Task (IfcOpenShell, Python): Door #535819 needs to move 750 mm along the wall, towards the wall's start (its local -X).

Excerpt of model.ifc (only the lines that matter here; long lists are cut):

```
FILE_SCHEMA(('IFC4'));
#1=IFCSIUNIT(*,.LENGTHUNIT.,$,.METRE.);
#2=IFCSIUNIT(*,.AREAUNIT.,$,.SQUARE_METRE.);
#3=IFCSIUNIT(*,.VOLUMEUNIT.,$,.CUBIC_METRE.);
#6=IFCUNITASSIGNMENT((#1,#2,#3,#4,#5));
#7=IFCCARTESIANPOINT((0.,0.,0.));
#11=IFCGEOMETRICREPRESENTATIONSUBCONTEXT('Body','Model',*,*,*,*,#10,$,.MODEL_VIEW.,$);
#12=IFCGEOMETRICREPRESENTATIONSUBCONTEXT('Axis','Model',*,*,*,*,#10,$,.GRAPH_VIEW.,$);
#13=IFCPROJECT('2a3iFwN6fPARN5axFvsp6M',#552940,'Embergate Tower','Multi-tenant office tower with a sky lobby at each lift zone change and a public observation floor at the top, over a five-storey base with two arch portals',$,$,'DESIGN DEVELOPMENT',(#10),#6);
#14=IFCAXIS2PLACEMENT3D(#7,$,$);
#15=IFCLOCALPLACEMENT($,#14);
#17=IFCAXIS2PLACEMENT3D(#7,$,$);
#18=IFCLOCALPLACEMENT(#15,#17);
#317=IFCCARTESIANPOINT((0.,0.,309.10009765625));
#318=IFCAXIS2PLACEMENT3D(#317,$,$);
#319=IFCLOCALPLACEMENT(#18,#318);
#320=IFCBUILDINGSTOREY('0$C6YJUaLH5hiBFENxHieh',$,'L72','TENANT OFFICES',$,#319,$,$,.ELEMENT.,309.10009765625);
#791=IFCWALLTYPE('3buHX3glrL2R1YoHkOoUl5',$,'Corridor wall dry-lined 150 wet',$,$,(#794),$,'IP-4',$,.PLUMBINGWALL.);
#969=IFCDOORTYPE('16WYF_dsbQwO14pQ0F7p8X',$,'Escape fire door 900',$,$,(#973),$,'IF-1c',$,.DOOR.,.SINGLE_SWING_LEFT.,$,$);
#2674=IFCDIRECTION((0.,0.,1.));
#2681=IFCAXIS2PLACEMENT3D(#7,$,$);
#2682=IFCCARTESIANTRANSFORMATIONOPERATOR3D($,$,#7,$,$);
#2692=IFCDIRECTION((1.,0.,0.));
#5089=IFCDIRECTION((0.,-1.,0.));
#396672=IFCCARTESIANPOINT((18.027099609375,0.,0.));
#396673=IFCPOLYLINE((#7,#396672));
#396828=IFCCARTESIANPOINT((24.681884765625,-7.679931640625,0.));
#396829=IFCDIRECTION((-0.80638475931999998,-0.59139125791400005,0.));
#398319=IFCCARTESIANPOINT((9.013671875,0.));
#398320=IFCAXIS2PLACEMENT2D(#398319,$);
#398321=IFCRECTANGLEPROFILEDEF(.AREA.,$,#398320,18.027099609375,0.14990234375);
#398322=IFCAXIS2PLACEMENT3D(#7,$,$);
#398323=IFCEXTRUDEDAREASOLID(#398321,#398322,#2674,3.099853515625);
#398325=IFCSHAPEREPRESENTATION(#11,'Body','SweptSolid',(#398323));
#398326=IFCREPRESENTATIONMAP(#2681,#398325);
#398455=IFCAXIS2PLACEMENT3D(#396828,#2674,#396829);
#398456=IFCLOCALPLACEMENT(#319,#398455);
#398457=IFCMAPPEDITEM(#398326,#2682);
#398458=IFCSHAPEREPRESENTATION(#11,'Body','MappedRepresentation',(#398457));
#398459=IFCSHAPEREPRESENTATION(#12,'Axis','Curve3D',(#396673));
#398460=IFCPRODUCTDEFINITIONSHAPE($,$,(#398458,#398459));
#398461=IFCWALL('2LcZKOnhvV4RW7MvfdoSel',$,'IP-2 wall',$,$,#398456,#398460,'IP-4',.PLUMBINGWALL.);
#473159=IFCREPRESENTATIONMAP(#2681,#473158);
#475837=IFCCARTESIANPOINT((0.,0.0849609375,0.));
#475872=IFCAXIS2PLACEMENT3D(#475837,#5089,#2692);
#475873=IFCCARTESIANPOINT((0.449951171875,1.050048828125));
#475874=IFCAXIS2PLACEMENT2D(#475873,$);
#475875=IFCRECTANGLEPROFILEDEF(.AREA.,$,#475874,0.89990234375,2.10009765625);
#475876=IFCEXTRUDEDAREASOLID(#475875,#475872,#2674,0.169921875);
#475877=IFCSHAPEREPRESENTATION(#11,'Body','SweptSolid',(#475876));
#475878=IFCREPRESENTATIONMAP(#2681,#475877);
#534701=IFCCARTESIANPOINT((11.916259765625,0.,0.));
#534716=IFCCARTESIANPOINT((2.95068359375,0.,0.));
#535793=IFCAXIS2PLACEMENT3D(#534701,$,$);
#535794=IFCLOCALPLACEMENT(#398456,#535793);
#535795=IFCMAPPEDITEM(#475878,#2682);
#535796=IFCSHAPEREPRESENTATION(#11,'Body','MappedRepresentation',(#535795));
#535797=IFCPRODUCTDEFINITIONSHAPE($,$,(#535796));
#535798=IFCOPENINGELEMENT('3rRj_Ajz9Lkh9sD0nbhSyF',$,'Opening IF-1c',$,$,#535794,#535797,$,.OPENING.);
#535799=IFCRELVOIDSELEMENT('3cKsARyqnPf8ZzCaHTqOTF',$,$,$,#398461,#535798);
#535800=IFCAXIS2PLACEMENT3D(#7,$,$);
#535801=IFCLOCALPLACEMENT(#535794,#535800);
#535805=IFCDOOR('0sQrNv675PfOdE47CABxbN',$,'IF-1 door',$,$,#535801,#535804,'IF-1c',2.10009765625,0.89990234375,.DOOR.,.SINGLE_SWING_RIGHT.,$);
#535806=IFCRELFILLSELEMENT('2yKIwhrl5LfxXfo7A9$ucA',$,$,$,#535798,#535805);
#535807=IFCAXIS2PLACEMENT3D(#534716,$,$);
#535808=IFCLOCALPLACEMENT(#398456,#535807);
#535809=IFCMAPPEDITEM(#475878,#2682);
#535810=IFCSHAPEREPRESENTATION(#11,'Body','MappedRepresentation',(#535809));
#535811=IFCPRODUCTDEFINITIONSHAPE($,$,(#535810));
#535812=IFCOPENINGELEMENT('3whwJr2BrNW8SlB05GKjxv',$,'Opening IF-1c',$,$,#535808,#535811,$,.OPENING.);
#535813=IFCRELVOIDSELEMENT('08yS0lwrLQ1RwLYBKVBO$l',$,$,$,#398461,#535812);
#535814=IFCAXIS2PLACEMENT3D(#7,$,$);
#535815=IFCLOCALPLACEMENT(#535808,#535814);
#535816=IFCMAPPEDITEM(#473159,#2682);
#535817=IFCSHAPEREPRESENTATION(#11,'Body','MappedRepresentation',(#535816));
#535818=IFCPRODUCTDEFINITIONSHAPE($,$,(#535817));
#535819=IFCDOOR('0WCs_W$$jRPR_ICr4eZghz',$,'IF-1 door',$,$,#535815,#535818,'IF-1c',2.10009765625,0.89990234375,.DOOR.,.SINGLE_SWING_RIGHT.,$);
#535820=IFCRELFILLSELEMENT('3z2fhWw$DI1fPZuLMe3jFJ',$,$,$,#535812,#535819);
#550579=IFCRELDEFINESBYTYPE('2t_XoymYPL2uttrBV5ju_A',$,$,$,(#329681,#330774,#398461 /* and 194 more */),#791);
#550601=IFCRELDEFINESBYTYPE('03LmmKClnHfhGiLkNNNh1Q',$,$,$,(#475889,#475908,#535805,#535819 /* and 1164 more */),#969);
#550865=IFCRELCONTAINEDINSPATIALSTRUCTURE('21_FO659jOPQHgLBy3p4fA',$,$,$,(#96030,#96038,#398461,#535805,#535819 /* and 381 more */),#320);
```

```python
import ifcopenshell
import ifcopenshell.api.geometry
import ifcopenshell.util.placement
import ifcopenshell.util.unit

model = ifcopenshell.open("model.ifc")
unit_scale = ifcopenshell.util.unit.calculate_unit_scale(model)

door = model.by_guid("0WCs_W$$jRPR_ICr4eZghz")
opening = door.FillsVoids[0].RelatingOpeningElement
wall = opening.VoidsElements[0].RelatingBuildingElement

wall_matrix = ifcopenshell.util.placement.get_local_placement(wall.ObjectPlacement)
shift = wall_matrix[:3, 0] * -0.75 / unit_scale
before = ifcopenshell.util.placement.get_local_placement(door.ObjectPlacement)[:3, 3].copy()

# The door is placed relative to its opening, so it follows when the opening moves.
matrix = ifcopenshell.util.placement.get_local_placement(opening.ObjectPlacement)
matrix[:3, 3] += shift
ifcopenshell.api.geometry.edit_object_placement(
    model, product=opening, matrix=matrix, is_si=False, should_transform_children=True
)

after = ifcopenshell.util.placement.get_local_placement(door.ObjectPlacement)[:3, 3]
print("door moved by", (after - before).round(3) + 0.0)

model.write("model_edited.ifc")
```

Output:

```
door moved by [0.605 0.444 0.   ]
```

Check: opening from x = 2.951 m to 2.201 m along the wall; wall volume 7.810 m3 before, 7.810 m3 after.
